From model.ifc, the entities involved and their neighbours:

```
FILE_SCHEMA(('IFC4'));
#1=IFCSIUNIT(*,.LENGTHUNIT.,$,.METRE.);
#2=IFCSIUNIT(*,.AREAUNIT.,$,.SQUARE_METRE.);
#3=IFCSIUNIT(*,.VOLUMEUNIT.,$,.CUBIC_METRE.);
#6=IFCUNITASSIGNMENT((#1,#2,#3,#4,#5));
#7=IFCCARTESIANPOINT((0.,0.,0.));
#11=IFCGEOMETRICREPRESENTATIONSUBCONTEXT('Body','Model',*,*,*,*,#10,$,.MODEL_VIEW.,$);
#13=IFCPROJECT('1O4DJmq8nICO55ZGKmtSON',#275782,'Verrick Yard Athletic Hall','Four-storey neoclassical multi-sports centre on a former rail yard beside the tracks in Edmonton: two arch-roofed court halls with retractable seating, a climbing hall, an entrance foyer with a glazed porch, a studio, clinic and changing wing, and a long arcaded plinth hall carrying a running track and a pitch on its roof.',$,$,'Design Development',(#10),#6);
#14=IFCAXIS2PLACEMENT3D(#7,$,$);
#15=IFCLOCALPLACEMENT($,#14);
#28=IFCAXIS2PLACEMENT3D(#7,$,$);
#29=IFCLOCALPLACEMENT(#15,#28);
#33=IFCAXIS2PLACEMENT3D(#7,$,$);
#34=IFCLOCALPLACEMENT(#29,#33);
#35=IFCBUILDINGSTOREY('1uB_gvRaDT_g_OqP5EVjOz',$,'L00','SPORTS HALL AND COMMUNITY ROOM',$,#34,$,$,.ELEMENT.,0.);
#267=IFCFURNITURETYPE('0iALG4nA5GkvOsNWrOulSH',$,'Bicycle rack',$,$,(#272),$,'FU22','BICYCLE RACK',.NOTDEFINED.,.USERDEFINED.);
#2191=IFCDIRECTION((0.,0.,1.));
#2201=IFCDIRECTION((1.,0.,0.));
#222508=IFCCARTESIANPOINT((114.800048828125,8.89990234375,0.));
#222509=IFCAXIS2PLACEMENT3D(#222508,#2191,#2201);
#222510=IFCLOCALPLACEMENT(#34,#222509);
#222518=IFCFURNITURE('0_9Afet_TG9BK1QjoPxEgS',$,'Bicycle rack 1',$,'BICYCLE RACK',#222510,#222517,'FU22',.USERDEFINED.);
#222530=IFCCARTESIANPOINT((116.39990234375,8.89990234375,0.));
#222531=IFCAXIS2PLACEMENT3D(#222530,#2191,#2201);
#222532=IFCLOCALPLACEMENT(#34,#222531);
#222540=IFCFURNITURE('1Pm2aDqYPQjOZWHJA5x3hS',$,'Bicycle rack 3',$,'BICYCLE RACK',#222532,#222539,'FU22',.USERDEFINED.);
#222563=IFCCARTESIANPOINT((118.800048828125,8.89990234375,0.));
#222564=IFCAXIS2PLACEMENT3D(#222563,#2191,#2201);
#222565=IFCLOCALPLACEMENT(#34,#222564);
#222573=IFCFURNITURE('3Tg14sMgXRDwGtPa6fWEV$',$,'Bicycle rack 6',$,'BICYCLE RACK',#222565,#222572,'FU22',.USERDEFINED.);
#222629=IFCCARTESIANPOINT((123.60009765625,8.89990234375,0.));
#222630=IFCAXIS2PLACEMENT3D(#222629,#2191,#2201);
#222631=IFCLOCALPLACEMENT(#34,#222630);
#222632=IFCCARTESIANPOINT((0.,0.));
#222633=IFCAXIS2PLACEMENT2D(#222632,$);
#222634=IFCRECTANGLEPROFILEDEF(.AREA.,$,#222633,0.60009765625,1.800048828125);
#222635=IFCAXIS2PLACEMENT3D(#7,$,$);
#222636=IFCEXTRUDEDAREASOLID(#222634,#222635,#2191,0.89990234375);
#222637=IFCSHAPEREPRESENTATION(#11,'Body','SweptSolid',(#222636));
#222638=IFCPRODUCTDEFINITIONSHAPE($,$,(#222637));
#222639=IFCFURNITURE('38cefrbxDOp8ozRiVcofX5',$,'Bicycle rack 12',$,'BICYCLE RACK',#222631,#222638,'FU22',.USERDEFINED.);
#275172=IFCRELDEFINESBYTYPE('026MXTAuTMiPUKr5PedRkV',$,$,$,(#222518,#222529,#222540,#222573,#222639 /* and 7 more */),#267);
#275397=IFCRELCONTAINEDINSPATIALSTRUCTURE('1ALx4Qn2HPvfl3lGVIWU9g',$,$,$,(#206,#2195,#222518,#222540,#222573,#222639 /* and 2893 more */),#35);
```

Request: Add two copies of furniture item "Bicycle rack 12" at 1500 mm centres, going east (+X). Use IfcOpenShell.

```python
import numpy as np
import ifcopenshell
import ifcopenshell.api.geometry
import ifcopenshell.api.root
import ifcopenshell.util.element
import ifcopenshell.util.placement

model = ifcopenshell.open("model.ifc")

source = model.by_id(222639)
base = ifcopenshell.util.placement.get_local_placement(source.ObjectPlacement)
step = np.array([1.0, 0.0, 0.0]) * 1.5

for i in range(1, 3):
    copy = ifcopenshell.api.root.copy_class(model, product=source)
    copy.Representation = ifcopenshell.util.element.copy_deep(
        model, source.Representation, exclude=["IfcGeometricRepresentationContext", "IfcRepresentationMap"]
    )
    copy.Tag = None
    matrix = base.copy()
    matrix[:3, 3] += i * step
    print("added at", matrix[:3, 3].round(3) + 0.0)
    ifcopenshell.api.geometry.edit_object_placement(model, product=copy, matrix=matrix, is_si=False)

model.write("model_v2.ifc")
```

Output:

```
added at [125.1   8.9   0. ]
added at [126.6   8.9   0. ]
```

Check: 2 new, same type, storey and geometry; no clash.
